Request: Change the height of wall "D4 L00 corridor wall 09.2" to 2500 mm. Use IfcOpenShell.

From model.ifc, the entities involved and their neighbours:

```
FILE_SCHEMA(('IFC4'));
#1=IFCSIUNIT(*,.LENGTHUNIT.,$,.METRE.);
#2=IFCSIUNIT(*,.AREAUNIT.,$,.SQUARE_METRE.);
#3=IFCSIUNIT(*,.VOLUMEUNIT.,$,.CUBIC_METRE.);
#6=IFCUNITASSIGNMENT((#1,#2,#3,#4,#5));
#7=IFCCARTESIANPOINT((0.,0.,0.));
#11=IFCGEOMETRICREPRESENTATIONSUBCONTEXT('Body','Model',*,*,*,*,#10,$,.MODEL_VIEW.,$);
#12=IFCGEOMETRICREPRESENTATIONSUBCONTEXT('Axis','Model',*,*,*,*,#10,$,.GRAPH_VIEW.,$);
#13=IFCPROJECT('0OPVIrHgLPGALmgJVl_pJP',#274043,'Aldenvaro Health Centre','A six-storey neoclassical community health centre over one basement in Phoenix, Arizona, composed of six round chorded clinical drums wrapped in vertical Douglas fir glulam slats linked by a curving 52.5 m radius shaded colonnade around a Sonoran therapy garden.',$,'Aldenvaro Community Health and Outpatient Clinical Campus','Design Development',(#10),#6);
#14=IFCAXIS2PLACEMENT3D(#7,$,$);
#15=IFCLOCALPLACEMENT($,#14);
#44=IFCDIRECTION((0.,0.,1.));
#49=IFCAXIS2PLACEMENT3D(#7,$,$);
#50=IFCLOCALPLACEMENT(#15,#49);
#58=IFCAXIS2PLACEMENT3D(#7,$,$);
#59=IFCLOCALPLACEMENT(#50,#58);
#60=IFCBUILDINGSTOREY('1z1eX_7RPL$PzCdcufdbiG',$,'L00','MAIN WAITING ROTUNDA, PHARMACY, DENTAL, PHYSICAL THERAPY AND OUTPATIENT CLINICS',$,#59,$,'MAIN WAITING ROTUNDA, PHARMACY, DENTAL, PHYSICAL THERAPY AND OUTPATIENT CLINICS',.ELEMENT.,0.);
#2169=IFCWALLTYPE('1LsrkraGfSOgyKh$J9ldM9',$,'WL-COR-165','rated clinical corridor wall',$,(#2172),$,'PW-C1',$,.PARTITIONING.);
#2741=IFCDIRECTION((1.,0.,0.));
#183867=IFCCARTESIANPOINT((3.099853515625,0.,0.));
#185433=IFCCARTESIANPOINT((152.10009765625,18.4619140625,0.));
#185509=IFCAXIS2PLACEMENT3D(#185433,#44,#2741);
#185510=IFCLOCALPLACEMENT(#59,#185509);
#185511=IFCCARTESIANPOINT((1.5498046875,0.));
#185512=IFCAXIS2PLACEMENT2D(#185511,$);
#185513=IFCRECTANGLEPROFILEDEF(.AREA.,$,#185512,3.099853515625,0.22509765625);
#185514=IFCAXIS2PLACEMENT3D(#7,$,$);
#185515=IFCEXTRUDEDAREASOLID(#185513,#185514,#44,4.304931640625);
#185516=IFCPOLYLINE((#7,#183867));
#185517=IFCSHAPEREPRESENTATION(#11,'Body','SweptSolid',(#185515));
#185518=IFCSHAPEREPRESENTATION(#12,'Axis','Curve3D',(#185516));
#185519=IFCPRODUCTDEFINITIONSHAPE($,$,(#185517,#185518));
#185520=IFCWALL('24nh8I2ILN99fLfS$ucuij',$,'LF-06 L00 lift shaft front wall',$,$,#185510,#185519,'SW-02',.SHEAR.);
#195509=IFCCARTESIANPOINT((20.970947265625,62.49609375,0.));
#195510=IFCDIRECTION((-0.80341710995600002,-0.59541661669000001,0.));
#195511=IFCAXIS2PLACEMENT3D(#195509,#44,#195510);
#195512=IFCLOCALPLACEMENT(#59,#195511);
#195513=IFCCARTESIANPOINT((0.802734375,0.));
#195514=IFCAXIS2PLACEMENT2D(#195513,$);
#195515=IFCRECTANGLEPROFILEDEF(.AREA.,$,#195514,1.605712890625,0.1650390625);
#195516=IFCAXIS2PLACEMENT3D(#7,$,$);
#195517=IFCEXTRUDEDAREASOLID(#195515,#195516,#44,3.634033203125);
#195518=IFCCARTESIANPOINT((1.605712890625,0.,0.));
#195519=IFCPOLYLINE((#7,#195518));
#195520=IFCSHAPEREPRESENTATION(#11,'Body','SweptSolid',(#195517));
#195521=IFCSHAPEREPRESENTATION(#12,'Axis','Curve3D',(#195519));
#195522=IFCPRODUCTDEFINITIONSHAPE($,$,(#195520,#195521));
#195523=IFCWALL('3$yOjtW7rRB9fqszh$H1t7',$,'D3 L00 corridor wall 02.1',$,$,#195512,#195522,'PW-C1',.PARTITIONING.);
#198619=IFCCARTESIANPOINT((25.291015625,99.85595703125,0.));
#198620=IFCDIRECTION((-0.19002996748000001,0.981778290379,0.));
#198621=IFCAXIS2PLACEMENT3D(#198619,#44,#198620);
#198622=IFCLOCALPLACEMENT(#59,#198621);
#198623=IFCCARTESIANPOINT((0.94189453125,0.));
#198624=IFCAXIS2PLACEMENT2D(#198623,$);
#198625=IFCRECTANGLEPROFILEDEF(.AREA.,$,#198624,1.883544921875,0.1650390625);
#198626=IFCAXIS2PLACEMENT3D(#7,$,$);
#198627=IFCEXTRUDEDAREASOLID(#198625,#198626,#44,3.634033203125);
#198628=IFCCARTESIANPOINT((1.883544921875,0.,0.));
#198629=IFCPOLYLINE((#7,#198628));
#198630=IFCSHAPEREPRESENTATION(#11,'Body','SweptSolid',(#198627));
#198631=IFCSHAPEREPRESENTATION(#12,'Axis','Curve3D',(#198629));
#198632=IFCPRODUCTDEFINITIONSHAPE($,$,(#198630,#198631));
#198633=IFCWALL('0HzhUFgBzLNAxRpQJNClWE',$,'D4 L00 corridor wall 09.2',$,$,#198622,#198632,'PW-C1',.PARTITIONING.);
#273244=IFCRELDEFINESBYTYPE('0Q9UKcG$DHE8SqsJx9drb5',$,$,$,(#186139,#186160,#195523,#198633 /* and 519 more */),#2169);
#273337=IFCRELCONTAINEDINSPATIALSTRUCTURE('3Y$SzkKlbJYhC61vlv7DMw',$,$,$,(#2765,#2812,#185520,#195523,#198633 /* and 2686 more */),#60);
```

```python
import ifcopenshell
import ifcopenshell.geom
import ifcopenshell.util.representation
import ifcopenshell.util.shape

model = ifcopenshell.open("model.ifc")
settings = ifcopenshell.geom.settings()


def volume(element):
    """Net volume in cubic metres, openings subtracted."""
    shape = ifcopenshell.geom.create_shape(settings, element)
    return ifcopenshell.util.shape.get_volume(shape.geometry)


wall = model.by_guid("0HzhUFgBzLNAxRpQJNClWE")
before = volume(wall)

body = ifcopenshell.util.representation.get_representation(wall, "Model", "Body")
solid = body.Items[0]
old_height = solid.Depth
solid.Depth = 2.5
after = volume(wall)

print(f"height {old_height:g} -> {solid.Depth:g}, volume {before:.3f} -> {after:.3f} m3")

model.write("model_updated.ifc")
```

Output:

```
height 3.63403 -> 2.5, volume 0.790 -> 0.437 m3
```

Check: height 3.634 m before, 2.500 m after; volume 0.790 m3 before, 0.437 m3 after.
